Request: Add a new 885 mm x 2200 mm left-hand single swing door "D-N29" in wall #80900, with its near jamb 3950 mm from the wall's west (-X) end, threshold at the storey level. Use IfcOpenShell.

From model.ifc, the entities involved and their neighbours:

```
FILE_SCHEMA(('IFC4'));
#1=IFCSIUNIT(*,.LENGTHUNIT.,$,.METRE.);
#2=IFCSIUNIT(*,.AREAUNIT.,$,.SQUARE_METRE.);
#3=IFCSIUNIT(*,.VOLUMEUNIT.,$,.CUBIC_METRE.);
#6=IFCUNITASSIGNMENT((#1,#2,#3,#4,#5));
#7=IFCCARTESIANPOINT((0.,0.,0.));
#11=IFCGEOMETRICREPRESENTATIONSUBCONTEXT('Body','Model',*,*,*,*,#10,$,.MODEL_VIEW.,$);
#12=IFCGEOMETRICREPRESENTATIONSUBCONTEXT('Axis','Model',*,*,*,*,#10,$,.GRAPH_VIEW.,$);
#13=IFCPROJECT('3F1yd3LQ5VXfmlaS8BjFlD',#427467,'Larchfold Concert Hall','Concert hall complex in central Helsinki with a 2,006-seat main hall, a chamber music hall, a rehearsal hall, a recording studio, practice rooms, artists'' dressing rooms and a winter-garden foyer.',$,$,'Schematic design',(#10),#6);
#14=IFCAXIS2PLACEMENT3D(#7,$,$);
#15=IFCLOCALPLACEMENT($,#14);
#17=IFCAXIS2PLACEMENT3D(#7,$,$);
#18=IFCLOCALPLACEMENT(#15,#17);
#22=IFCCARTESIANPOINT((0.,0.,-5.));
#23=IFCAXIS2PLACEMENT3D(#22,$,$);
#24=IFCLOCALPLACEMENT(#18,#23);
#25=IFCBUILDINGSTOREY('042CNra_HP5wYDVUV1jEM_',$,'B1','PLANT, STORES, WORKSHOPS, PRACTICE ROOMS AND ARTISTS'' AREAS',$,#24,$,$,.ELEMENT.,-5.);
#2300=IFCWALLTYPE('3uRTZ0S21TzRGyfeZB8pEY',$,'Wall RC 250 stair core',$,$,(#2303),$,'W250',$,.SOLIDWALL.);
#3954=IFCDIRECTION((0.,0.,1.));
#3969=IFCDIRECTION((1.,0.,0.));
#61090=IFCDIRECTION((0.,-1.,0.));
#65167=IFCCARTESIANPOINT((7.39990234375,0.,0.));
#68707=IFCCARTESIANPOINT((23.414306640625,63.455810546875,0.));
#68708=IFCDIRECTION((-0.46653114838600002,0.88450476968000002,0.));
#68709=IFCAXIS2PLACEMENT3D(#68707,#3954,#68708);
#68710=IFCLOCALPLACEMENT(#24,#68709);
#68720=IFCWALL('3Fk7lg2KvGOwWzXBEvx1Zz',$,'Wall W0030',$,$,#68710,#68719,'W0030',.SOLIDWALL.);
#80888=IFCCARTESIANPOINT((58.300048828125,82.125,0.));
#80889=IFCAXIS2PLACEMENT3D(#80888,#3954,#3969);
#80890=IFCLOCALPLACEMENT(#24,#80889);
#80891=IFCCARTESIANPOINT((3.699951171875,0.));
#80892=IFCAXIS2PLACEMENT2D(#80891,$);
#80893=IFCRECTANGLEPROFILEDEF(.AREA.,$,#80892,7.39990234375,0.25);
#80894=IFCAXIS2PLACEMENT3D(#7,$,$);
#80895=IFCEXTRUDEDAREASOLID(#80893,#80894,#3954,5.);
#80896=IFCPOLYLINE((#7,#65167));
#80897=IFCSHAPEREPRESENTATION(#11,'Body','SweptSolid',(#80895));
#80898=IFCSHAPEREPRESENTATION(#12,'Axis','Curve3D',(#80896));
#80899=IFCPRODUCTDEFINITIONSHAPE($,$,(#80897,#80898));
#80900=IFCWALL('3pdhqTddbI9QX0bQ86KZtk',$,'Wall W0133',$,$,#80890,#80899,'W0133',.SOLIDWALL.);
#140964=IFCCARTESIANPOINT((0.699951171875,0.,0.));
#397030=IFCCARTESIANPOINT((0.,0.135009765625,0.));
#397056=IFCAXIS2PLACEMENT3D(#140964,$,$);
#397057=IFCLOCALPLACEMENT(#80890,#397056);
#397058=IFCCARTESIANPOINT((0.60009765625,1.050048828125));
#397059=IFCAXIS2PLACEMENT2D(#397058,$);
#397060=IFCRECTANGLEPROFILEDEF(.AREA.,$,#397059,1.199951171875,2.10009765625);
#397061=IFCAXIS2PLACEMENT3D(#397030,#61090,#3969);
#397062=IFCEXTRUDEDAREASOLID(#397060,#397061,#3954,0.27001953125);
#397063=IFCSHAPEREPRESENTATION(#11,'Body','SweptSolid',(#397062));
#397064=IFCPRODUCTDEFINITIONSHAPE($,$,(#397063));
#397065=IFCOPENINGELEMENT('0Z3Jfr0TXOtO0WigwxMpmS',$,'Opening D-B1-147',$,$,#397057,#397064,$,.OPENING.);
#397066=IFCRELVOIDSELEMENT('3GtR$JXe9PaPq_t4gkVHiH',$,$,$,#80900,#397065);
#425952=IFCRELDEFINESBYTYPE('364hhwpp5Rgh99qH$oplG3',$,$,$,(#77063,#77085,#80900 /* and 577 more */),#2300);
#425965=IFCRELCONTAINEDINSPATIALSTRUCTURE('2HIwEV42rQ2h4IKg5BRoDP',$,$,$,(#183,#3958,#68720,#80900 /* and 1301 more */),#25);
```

```python
import numpy as np
import ifcopenshell
import ifcopenshell.api.feature
import ifcopenshell.api.geometry
import ifcopenshell.api.root
import ifcopenshell.api.spatial
import ifcopenshell.geom
import ifcopenshell.util.element
import ifcopenshell.util.placement
import ifcopenshell.util.representation
import ifcopenshell.util.shape
import ifcopenshell.util.unit

model = ifcopenshell.open("model.ifc")
unit_scale = ifcopenshell.util.unit.calculate_unit_scale(model)
settings = ifcopenshell.geom.settings()


def volume(element):
    """Net volume in cubic metres, openings subtracted."""
    shape = ifcopenshell.geom.create_shape(settings, element)
    return ifcopenshell.util.shape.get_volume(shape.geometry)


wall = model.by_id(80900)
storey = ifcopenshell.util.element.get_container(wall, ifc_class="IfcBuildingStorey")
context = ifcopenshell.util.representation.get_context(model, "Model", "Body", "MODEL_VIEW")
before = volume(wall)

width, height, from_end, sill = 0.885, 2.2, 3.95, 0.0  # metres

# The wall runs along its own X axis, and the end named is its -X end.
wall_shape = ifcopenshell.geom.create_shape(settings, wall)
x, y, z = ifcopenshell.util.shape.get_vertices(wall_shape.geometry).T
start = x.min() + from_end
face, thickness = float(y.min()), float(y.max() - y.min())
wall_matrix = ifcopenshell.util.placement.get_local_placement(wall.ObjectPlacement)
level = ifcopenshell.util.placement.get_local_placement(storey.ObjectPlacement)[2, 3]


def in_wall(x, y):
    """Placement at x, y metres in the wall's axes, at sill height."""
    matrix = wall_matrix.copy()
    matrix[:, 3] = wall_matrix @ np.array([x / unit_scale, y / unit_scale, 0.0, 1.0])
    matrix[2, 3] = level + sill / unit_scale
    return matrix


# Opening: a box that overshoots both wall faces by 50 mm.
opening = ifcopenshell.api.root.create_entity(model, ifc_class="IfcOpeningElement", predefined_type="OPENING")
box = ifcopenshell.api.geometry.add_wall_representation(
    model, context=context, length=width, height=height, thickness=thickness + 0.1
)
ifcopenshell.api.geometry.assign_representation(model, product=opening, representation=box)
ifcopenshell.api.geometry.edit_object_placement(model, product=opening, matrix=in_wall(start, face - 0.05), is_si=False)
ifcopenshell.api.feature.add_feature(model, feature=opening, element=wall)

door = ifcopenshell.api.root.create_entity(model, ifc_class="IfcDoor", name="D-N29", predefined_type="DOOR")
door.OverallWidth, door.OverallHeight = width / unit_scale, height / unit_scale
door.OperationType = "SINGLE_SWING_LEFT"
body = ifcopenshell.api.geometry.add_door_representation(
    model,
    context=context,
    overall_width=door.OverallWidth,
    overall_height=door.OverallHeight,
    operation_type="SINGLE_SWING_LEFT",
    lining_properties={"LiningDepth": thickness / unit_scale, "ThresholdDepth": thickness / unit_scale},
)
ifcopenshell.api.geometry.assign_representation(model, product=door, representation=body)
ifcopenshell.api.spatial.assign_container(model, products=[door], relating_structure=storey)
ifcopenshell.api.feature.add_filling(model, opening=opening, element=door)

# The lining spans the wall, so the door starts at the wall face.
ifcopenshell.api.geometry.edit_object_placement(model, product=door, matrix=in_wall(start, face), is_si=False)

after = volume(wall)

print(f"wall volume {before:.3f} -> {after:.3f} m3")

model.write("model_v2.ifc")
```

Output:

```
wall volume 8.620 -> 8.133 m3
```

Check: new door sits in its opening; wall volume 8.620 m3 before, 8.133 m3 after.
